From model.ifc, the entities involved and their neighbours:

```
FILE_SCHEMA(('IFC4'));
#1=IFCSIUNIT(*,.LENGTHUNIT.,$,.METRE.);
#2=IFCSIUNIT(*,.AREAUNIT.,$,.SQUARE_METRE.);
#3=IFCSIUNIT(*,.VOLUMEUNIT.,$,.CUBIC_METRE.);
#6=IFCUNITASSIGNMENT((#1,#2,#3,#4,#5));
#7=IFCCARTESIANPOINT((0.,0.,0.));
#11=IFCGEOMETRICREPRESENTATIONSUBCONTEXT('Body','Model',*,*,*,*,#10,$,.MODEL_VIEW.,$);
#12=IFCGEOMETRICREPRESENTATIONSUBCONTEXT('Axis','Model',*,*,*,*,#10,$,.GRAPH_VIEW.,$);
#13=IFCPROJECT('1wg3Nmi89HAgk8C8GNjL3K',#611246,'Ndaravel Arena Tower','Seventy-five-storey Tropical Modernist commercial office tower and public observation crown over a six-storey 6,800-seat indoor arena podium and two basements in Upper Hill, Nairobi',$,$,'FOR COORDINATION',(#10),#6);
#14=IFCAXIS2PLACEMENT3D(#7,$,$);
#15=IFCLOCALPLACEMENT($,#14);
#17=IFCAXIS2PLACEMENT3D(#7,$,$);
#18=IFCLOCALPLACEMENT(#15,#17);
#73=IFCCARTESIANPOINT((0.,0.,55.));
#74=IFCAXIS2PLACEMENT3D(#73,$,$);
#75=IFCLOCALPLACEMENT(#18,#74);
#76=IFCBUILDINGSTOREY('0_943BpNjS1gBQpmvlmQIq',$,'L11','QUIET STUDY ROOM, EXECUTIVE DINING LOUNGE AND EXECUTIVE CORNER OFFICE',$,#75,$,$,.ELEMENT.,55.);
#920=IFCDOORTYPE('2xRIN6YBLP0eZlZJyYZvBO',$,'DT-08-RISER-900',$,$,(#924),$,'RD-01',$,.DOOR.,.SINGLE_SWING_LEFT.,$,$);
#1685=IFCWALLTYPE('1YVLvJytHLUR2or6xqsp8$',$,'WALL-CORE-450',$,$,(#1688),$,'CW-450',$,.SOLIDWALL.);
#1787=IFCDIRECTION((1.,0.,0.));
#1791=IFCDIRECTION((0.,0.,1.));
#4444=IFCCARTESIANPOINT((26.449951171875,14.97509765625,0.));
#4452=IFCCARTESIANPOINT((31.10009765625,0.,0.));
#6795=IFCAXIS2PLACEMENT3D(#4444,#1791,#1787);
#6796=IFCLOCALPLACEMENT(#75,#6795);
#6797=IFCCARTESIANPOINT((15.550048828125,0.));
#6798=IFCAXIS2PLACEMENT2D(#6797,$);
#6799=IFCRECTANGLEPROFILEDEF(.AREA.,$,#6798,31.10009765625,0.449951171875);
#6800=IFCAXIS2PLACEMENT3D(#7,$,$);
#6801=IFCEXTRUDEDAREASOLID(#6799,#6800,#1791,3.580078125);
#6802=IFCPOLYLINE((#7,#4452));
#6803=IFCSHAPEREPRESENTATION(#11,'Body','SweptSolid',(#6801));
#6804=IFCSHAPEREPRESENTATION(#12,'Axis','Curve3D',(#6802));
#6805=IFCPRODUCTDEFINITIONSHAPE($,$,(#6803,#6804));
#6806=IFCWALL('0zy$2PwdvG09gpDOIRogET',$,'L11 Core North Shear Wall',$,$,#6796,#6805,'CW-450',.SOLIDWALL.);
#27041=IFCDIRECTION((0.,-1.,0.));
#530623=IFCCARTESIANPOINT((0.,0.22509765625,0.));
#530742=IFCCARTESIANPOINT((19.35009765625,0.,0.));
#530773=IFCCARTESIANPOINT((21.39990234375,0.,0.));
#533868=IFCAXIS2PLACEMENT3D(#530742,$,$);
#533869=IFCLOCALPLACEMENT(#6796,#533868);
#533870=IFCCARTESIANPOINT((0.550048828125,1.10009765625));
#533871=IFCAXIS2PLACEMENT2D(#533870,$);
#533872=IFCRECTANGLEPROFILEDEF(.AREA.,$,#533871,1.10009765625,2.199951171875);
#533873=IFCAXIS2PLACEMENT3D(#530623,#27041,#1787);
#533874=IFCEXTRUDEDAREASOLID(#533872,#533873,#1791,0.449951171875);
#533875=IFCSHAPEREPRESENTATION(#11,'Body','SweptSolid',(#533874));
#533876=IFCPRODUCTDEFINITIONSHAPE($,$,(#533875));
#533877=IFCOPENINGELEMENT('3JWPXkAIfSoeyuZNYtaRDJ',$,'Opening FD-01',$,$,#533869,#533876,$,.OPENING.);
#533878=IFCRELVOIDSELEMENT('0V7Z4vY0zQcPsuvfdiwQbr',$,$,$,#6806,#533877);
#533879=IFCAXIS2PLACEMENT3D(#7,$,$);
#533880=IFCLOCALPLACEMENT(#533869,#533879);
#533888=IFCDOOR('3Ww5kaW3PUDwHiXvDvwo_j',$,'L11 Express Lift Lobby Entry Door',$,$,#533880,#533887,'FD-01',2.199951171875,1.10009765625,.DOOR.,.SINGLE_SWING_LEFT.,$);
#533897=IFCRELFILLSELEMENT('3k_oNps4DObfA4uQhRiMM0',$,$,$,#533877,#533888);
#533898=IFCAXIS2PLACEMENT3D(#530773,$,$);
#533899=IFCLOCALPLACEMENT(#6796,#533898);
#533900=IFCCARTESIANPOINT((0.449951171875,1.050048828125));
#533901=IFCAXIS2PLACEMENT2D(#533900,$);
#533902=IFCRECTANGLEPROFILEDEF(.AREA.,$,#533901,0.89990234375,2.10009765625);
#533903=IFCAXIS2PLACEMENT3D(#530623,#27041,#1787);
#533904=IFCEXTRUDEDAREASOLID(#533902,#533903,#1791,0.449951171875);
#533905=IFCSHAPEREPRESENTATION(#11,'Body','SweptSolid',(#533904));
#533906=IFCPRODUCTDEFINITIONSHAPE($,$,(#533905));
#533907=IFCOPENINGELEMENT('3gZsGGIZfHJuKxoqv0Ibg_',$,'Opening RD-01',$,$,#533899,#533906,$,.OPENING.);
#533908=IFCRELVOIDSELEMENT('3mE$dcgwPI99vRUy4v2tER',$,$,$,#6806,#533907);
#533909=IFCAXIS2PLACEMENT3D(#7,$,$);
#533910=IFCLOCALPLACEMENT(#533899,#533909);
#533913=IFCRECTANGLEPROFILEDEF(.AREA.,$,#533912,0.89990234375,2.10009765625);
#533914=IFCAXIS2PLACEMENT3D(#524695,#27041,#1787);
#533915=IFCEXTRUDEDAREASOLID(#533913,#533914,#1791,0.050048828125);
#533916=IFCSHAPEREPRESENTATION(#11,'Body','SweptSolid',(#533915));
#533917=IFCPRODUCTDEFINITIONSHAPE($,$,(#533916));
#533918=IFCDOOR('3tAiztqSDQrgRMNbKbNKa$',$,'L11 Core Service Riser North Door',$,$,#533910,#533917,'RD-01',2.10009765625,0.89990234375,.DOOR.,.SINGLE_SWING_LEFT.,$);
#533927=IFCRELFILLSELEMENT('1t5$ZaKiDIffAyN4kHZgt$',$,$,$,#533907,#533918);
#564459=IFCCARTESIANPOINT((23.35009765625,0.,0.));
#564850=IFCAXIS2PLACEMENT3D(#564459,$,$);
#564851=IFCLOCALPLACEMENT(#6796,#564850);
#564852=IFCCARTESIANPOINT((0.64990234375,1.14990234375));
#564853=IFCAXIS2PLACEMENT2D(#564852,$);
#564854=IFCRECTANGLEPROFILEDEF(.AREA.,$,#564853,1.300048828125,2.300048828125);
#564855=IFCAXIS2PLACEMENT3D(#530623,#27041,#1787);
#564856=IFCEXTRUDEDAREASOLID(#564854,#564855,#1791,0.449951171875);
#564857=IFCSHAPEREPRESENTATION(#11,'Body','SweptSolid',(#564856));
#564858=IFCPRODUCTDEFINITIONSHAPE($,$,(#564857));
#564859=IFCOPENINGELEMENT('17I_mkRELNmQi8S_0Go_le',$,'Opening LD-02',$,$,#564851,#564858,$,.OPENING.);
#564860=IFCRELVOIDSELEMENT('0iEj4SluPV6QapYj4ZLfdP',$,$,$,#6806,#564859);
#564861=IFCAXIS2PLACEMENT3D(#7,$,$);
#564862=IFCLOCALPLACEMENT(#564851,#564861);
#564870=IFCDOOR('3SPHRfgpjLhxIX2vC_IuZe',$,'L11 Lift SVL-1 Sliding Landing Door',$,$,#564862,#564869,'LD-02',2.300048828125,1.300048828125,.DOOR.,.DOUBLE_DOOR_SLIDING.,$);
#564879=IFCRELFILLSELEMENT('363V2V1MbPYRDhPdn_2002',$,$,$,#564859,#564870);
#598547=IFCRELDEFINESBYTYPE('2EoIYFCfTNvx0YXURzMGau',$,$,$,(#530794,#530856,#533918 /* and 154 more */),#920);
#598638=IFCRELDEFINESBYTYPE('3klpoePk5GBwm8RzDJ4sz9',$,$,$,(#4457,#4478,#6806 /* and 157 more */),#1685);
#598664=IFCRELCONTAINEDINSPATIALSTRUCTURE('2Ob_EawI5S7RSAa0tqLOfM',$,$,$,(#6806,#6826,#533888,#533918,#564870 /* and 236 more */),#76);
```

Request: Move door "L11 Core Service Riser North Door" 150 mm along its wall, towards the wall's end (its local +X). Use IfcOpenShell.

```python
import ifcopenshell
import ifcopenshell.api.geometry
import ifcopenshell.util.placement

model = ifcopenshell.open("model.ifc")

door = model.by_guid("3tAiztqSDQrgRMNbKbNKa$")
opening = door.FillsVoids[0].RelatingOpeningElement
wall = opening.VoidsElements[0].RelatingBuildingElement

wall_matrix = ifcopenshell.util.placement.get_local_placement(wall.ObjectPlacement)
shift = wall_matrix[:3, 0] * 0.15
before = ifcopenshell.util.placement.get_local_placement(door.ObjectPlacement)[:3, 3].copy()

# The door is placed relative to its opening, so it follows when the opening moves.
matrix = ifcopenshell.util.placement.get_local_placement(opening.ObjectPlacement)
matrix[:3, 3] += shift
ifcopenshell.api.geometry.edit_object_placement(
    model, product=opening, matrix=matrix, is_si=False, should_transform_children=True
)

after = ifcopenshell.util.placement.get_local_placement(door.ObjectPlacement)[:3, 3]
print("door moved by", (after - before).round(3) + 0.0)

model.write("model_edited.ifc")
```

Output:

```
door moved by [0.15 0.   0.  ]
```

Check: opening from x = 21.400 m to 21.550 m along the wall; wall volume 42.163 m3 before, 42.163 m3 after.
